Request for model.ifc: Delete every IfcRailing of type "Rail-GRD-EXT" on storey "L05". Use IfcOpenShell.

First a look at what the model holds.

```python
import ifcopenshell
import ifcopenshell.util.element

model = ifcopenshell.open("model.ifc")
print(model.schema)
storey = next(s for s in model.by_type("IfcBuildingStorey") if s.Name == "L05")
railings = [e for e in ifcopenshell.util.element.get_decomposition(storey) if e.is_a("IfcRailing")]
seen = {}
for e in railings:
    element_type = ifcopenshell.util.element.get_type(e)
    name = element_type.Name if element_type not in (None, e) else None
    seen[name] = seen.get(name, 0) + 1
for name, count in sorted(seen.items(), key=str):
    print(count, "x", name)
```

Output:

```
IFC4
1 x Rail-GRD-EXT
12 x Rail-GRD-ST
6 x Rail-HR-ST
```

```python
import ifcopenshell
import ifcopenshell.api.root
import ifcopenshell.util.element

model = ifcopenshell.open("model.ifc")

storey = next(s for s in model.by_type("IfcBuildingStorey") if s.Name == "L05")
railings = [e for e in ifcopenshell.util.element.get_decomposition(storey) if e.is_a("IfcRailing")]
targets = [e for e in railings if (t := ifcopenshell.util.element.get_type(e)) not in (None, e) and t.Name == "Rail-GRD-EXT"]

for e in targets:
    ifcopenshell.api.root.remove_product(model, product=e)
print(len(targets), "removed")

model.write("model_updated.ifc")
```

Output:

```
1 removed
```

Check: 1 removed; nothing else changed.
